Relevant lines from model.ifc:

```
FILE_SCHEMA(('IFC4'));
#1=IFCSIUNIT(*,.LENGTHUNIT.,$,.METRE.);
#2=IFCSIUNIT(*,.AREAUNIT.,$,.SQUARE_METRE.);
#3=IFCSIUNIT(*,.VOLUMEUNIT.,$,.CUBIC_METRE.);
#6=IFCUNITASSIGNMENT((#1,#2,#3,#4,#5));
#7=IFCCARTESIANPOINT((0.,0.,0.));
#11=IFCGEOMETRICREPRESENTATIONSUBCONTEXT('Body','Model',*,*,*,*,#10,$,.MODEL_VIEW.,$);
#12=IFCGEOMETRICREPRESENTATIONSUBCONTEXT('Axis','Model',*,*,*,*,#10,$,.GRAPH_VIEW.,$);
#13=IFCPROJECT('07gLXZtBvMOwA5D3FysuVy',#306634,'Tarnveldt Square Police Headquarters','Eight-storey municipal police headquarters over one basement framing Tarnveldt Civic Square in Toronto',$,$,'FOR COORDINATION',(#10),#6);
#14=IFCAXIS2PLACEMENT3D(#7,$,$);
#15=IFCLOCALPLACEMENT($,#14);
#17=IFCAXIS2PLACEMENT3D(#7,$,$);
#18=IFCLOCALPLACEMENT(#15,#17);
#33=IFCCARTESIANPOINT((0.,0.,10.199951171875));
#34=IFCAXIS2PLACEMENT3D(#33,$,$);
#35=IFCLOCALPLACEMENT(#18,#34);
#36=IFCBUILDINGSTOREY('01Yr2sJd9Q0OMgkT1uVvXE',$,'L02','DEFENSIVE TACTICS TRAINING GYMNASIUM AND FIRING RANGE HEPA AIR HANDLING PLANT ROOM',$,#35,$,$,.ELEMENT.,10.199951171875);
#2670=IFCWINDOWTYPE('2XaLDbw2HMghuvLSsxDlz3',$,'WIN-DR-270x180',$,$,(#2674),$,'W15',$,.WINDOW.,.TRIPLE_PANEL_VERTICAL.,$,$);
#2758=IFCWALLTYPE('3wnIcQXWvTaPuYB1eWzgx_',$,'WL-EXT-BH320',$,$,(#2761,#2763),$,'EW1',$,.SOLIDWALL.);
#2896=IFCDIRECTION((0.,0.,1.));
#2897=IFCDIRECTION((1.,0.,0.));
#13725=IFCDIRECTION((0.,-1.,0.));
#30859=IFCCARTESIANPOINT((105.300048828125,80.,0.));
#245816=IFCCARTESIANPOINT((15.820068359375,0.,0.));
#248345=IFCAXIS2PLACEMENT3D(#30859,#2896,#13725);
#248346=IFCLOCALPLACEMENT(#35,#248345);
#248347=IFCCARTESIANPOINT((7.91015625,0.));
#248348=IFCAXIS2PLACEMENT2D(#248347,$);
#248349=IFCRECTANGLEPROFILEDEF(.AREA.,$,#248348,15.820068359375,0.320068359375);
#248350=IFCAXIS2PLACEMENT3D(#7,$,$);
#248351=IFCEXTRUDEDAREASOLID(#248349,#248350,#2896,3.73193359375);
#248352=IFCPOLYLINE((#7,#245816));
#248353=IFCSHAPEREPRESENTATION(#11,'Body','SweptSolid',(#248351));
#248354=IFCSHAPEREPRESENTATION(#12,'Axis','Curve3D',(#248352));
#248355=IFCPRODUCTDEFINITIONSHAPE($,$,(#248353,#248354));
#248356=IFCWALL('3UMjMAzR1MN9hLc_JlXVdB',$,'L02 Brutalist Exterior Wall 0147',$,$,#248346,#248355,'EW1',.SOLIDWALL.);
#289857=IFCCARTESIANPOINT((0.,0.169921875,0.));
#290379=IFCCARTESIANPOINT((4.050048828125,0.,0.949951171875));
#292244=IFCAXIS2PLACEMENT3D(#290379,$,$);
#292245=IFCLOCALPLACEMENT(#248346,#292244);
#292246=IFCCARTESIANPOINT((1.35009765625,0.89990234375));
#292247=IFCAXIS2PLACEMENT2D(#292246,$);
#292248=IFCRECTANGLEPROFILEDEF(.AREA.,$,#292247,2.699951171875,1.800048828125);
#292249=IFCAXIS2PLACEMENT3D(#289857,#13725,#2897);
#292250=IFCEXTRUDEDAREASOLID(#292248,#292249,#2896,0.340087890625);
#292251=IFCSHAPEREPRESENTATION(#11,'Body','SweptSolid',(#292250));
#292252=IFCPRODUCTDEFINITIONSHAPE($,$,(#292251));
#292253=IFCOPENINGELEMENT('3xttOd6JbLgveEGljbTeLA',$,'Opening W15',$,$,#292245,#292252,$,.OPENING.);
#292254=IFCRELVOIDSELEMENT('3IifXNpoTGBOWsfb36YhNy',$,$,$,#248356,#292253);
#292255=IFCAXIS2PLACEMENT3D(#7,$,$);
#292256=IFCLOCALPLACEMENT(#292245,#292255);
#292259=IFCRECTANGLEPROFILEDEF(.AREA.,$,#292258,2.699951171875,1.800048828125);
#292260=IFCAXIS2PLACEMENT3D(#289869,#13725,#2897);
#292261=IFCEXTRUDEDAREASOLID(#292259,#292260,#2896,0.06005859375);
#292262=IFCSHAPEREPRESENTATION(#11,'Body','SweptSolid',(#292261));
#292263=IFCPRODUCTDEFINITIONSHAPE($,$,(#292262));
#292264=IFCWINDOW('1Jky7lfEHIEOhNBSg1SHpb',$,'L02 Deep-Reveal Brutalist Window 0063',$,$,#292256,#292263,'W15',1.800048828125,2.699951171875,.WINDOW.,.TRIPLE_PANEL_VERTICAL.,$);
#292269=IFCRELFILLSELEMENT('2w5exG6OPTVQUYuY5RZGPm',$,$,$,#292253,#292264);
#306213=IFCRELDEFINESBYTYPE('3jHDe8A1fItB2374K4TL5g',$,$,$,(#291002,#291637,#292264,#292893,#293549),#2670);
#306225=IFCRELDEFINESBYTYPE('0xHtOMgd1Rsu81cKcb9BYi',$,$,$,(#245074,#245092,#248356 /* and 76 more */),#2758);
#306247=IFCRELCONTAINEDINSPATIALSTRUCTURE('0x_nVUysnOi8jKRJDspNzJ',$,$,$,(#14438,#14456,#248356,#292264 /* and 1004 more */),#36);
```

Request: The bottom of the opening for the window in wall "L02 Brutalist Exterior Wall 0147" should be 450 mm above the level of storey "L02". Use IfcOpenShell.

```python
import numpy as np
import ifcopenshell
import ifcopenshell.api.geometry
import ifcopenshell.geom
import ifcopenshell.util.element
import ifcopenshell.util.placement
import ifcopenshell.util.shape
import ifcopenshell.util.unit

model = ifcopenshell.open("model.ifc")
unit_scale = ifcopenshell.util.unit.calculate_unit_scale(model)

window = model.by_id(292264)
opening = window.FillsVoids[0].RelatingOpeningElement
storey = ifcopenshell.util.element.get_container(window, ifc_class="IfcBuildingStorey")
level = ifcopenshell.util.placement.get_local_placement(storey.ObjectPlacement)[2, 3]

# The opening's origin need not be at the sill, so measure its lowest point.
shape = ifcopenshell.geom.create_shape(ifcopenshell.geom.settings(), opening)
bottom = ifcopenshell.util.shape.get_shape_bottom_elevation(shape, shape.geometry) / unit_scale
dz = level + 0.45 - bottom

shift = np.array([0.0, 0.0, dz])
# The window is placed relative to its opening, so it follows when the opening moves.
matrix = ifcopenshell.util.placement.get_local_placement(opening.ObjectPlacement)
matrix[:3, 3] += shift
ifcopenshell.api.geometry.edit_object_placement(
    model, product=opening, matrix=matrix, is_si=False, should_transform_children=True
)

print(f"moved by {dz * unit_scale:+.3f} m")

model.write("model_updated.ifc")
```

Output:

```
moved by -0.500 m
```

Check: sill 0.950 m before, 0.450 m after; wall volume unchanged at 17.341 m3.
